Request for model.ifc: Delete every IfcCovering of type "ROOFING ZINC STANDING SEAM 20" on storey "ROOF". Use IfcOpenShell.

First a look at what the model holds.

```python
import ifcopenshell
import ifcopenshell.util.element

model = ifcopenshell.open("model.ifc")
print(model.schema)
storey = next(s for s in model.by_type("IfcBuildingStorey") if s.Name == "ROOF")
coverings = [e for e in ifcopenshell.util.element.get_decomposition(storey) if e.is_a("IfcCovering")]
seen = {}
for e in coverings:
    element_type = ifcopenshell.util.element.get_type(e)
    name = element_type.Name if element_type not in (None, e) else None
    seen[name] = seen.get(name, 0) + 1
for name, count in sorted(seen.items(), key=str):
    print(count, "x", name)
```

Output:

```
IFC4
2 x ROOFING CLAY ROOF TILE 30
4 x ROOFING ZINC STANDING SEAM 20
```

```python
import ifcopenshell
import ifcopenshell.api.root
import ifcopenshell.util.element

model = ifcopenshell.open("model.ifc")

storey = next(s for s in model.by_type("IfcBuildingStorey") if s.Name == "ROOF")
coverings = [e for e in ifcopenshell.util.element.get_decomposition(storey) if e.is_a("IfcCovering")]
targets = [e for e in coverings if (t := ifcopenshell.util.element.get_type(e)) not in (None, e) and t.Name == "ROOFING ZINC STANDING SEAM 20"]

for e in targets:
    ifcopenshell.api.root.remove_product(model, product=e)
print(len(targets), "removed")

model.write("model_edited.ifc")
```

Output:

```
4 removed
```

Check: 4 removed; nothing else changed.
